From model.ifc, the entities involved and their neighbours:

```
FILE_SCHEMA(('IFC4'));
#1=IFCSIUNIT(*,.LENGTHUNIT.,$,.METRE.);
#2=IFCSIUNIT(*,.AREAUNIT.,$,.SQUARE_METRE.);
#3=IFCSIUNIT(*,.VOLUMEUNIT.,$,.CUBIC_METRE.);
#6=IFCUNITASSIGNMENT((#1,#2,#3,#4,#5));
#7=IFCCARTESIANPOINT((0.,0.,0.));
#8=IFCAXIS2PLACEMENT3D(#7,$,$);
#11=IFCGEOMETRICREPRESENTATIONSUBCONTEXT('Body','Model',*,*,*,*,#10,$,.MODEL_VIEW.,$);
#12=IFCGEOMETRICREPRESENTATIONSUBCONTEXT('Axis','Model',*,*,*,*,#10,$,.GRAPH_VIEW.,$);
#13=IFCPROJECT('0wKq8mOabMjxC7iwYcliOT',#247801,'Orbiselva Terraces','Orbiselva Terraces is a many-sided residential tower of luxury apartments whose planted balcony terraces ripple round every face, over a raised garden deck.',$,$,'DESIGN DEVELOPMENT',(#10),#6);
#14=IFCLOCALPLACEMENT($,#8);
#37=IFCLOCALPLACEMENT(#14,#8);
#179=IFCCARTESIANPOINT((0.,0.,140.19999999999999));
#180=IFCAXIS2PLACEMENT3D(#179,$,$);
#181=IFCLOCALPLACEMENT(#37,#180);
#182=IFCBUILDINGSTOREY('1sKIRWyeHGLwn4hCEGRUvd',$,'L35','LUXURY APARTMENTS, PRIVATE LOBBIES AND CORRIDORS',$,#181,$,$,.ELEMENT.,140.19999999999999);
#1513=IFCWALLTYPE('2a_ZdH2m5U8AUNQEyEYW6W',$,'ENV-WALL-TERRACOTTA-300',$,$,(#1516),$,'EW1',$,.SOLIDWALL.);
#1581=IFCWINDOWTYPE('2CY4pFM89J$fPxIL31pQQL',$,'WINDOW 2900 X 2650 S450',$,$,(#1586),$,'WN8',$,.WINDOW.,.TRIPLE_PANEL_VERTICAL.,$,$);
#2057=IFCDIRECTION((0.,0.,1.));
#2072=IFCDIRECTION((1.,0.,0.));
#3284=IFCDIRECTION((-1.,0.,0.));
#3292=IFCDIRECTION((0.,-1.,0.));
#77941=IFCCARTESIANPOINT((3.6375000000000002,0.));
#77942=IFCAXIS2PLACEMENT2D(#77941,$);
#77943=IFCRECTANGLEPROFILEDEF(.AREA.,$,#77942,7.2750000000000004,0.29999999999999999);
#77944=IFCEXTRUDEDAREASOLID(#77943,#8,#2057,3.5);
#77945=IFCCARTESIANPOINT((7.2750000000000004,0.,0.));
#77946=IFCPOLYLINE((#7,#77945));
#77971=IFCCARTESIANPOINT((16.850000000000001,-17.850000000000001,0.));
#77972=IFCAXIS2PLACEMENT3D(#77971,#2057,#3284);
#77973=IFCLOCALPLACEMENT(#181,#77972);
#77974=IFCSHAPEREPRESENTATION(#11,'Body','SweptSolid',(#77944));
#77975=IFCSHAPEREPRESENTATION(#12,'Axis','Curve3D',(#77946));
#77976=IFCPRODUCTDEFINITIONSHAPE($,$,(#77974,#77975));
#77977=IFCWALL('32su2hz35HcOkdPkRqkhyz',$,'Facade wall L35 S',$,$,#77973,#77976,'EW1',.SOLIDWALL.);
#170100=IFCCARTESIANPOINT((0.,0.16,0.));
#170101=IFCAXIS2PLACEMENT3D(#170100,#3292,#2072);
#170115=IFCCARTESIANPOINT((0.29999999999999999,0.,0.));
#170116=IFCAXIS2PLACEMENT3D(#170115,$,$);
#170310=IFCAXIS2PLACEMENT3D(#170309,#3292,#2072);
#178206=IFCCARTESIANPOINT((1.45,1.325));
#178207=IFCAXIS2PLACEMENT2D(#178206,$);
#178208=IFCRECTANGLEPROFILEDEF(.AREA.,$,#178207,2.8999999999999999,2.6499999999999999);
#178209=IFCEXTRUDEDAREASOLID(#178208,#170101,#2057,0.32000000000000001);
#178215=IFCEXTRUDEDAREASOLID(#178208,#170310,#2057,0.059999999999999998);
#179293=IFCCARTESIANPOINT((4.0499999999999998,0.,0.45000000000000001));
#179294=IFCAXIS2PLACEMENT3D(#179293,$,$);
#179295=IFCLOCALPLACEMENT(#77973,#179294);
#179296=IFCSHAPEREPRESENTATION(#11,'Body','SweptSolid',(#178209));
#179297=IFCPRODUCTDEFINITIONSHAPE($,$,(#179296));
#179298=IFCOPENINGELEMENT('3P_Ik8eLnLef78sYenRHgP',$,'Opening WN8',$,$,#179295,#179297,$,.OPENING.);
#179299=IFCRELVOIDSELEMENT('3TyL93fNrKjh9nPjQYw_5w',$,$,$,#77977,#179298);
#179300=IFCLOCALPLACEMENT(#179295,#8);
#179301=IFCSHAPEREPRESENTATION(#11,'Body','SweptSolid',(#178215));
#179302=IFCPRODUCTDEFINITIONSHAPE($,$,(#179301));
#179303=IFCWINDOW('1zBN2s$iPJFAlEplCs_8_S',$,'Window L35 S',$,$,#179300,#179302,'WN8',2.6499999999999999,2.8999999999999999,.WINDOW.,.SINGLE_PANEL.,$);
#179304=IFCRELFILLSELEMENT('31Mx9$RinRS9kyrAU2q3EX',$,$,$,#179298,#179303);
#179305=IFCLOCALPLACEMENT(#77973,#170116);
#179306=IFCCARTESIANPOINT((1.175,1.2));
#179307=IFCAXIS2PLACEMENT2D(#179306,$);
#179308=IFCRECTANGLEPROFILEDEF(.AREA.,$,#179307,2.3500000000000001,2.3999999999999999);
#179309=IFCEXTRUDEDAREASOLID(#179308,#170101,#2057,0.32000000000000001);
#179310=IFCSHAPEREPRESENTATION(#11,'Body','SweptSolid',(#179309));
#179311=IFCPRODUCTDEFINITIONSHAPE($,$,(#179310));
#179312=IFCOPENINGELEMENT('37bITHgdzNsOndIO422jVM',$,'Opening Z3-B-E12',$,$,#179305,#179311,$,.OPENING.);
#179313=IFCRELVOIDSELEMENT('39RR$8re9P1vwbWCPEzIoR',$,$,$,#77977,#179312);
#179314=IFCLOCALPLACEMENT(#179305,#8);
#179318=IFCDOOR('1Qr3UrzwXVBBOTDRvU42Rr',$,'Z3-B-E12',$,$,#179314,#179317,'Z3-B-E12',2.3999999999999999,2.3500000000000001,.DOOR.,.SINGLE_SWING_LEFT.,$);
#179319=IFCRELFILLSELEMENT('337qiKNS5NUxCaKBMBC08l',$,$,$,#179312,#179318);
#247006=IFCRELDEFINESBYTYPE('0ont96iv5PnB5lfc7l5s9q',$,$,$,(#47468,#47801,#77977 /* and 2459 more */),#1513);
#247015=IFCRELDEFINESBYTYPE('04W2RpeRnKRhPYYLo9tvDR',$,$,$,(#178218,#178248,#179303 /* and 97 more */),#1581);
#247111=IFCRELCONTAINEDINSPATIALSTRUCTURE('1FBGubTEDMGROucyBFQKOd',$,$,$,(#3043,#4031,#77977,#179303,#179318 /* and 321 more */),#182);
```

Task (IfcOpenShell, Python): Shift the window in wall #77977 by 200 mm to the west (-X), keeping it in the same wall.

```python
import ifcopenshell
import ifcopenshell.api.geometry
import ifcopenshell.util.placement

model = ifcopenshell.open("model.ifc")

window = model.by_guid("1zBN2s$iPJFAlEplCs_8_S")
opening = window.FillsVoids[0].RelatingOpeningElement
wall = opening.VoidsElements[0].RelatingBuildingElement

wall_matrix = ifcopenshell.util.placement.get_local_placement(wall.ObjectPlacement)
shift = wall_matrix[:3, 0] * 0.2
before = ifcopenshell.util.placement.get_local_placement(window.ObjectPlacement)[:3, 3].copy()

# The window is placed relative to its opening, so it follows when the opening moves.
matrix = ifcopenshell.util.placement.get_local_placement(opening.ObjectPlacement)
matrix[:3, 3] += shift
ifcopenshell.api.geometry.edit_object_placement(
    model, product=opening, matrix=matrix, is_si=False, should_transform_children=True
)

after = ifcopenshell.util.placement.get_local_placement(window.ObjectPlacement)[:3, 3]
print("window moved by", (after - before).round(3) + 0.0)

model.write("model_rev.ifc")
```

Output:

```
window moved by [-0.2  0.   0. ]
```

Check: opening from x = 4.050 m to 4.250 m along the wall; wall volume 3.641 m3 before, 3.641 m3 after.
